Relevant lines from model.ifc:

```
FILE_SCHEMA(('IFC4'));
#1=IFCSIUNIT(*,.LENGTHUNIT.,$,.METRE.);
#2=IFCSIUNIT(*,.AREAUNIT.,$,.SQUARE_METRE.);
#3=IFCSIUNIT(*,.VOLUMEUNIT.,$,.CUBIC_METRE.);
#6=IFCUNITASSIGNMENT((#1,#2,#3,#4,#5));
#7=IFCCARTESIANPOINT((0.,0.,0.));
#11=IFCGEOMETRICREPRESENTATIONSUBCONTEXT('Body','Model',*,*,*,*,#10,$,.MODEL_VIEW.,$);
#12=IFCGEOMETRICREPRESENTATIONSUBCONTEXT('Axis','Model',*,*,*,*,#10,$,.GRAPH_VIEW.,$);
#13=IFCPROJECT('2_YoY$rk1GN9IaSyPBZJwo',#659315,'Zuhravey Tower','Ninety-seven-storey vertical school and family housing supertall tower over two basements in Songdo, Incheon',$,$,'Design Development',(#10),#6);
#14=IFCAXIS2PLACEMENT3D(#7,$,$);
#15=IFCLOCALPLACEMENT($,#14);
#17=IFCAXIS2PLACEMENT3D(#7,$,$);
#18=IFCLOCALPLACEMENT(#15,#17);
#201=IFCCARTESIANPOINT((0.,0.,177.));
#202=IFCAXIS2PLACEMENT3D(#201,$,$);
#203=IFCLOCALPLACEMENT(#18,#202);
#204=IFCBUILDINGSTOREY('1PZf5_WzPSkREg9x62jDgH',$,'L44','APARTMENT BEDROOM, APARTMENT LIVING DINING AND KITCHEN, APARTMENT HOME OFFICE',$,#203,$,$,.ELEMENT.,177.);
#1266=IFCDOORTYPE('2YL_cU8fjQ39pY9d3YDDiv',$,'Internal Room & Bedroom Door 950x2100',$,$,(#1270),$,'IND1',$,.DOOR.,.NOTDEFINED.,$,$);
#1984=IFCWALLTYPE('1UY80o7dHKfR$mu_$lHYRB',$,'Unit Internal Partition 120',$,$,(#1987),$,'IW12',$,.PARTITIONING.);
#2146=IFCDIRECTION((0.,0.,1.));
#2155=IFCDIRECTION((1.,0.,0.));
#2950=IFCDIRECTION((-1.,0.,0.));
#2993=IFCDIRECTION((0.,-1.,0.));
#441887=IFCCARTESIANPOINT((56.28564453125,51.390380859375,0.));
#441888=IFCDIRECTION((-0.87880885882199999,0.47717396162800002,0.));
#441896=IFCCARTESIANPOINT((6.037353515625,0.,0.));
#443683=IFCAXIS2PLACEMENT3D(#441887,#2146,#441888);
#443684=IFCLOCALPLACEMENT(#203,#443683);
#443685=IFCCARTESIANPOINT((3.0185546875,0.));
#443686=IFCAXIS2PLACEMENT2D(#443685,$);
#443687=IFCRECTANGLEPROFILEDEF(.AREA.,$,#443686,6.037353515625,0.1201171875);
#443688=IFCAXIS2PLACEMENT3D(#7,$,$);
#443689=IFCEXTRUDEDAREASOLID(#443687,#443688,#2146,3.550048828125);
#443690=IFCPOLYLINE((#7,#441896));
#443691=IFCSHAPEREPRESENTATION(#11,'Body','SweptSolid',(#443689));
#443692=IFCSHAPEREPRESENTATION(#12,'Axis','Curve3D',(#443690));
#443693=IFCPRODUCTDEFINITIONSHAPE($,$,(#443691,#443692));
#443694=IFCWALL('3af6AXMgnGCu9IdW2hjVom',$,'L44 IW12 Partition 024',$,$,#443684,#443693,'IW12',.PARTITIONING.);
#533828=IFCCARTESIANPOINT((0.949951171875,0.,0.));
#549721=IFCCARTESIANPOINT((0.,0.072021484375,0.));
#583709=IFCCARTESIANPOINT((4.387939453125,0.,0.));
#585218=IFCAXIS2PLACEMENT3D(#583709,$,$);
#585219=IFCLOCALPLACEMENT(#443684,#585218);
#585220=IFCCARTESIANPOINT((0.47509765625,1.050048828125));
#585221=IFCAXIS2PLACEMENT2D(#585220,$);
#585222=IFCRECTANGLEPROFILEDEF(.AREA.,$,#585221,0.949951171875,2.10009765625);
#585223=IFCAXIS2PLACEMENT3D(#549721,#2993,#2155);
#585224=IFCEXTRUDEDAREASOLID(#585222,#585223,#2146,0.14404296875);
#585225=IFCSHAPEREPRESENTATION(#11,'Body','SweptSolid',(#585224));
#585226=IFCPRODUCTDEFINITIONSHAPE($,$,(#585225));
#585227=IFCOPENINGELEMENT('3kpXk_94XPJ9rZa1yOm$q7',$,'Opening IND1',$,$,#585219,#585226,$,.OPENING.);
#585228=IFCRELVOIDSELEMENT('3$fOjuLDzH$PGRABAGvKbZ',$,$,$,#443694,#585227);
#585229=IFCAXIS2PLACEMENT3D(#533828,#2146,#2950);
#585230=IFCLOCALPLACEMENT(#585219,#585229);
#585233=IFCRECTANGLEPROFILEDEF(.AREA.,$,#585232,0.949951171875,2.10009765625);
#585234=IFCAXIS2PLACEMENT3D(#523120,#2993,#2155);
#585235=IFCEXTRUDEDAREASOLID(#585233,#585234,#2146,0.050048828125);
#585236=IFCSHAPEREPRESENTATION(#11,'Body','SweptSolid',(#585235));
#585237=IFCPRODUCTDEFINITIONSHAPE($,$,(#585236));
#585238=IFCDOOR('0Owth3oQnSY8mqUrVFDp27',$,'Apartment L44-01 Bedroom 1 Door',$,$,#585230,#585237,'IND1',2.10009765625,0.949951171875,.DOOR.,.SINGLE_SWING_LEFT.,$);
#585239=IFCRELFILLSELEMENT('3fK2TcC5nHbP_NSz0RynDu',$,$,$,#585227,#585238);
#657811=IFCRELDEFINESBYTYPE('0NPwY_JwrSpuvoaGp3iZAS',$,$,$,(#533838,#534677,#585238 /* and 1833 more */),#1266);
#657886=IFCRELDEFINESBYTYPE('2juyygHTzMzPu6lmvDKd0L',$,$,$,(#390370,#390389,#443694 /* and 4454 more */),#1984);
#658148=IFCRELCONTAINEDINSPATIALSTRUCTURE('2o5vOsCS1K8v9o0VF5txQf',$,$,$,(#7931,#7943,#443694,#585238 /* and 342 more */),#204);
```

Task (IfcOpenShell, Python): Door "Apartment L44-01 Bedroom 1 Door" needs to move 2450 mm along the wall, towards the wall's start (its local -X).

```python
import ifcopenshell
import ifcopenshell.api.geometry
import ifcopenshell.util.placement
import ifcopenshell.util.unit

model = ifcopenshell.open("model.ifc")
unit_scale = ifcopenshell.util.unit.calculate_unit_scale(model)

door = model.by_guid("0Owth3oQnSY8mqUrVFDp27")
opening = door.FillsVoids[0].RelatingOpeningElement
wall = opening.VoidsElements[0].RelatingBuildingElement

wall_matrix = ifcopenshell.util.placement.get_local_placement(wall.ObjectPlacement)
shift = wall_matrix[:3, 0] * -2.45 / unit_scale
before = ifcopenshell.util.placement.get_local_placement(door.ObjectPlacement)[:3, 3].copy()

# The door is placed relative to its opening, so it follows when the opening moves.
matrix = ifcopenshell.util.placement.get_local_placement(opening.ObjectPlacement)
matrix[:3, 3] += shift
ifcopenshell.api.geometry.edit_object_placement(
    model, product=opening, matrix=matrix, is_si=False, should_transform_children=True
)

after = ifcopenshell.util.placement.get_local_placement(door.ObjectPlacement)[:3, 3]
print("door moved by", (after - before).round(3) + 0.0)

model.write("model_rev.ifc")
```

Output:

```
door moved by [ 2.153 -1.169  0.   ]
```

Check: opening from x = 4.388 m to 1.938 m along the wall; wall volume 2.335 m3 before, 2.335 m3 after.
